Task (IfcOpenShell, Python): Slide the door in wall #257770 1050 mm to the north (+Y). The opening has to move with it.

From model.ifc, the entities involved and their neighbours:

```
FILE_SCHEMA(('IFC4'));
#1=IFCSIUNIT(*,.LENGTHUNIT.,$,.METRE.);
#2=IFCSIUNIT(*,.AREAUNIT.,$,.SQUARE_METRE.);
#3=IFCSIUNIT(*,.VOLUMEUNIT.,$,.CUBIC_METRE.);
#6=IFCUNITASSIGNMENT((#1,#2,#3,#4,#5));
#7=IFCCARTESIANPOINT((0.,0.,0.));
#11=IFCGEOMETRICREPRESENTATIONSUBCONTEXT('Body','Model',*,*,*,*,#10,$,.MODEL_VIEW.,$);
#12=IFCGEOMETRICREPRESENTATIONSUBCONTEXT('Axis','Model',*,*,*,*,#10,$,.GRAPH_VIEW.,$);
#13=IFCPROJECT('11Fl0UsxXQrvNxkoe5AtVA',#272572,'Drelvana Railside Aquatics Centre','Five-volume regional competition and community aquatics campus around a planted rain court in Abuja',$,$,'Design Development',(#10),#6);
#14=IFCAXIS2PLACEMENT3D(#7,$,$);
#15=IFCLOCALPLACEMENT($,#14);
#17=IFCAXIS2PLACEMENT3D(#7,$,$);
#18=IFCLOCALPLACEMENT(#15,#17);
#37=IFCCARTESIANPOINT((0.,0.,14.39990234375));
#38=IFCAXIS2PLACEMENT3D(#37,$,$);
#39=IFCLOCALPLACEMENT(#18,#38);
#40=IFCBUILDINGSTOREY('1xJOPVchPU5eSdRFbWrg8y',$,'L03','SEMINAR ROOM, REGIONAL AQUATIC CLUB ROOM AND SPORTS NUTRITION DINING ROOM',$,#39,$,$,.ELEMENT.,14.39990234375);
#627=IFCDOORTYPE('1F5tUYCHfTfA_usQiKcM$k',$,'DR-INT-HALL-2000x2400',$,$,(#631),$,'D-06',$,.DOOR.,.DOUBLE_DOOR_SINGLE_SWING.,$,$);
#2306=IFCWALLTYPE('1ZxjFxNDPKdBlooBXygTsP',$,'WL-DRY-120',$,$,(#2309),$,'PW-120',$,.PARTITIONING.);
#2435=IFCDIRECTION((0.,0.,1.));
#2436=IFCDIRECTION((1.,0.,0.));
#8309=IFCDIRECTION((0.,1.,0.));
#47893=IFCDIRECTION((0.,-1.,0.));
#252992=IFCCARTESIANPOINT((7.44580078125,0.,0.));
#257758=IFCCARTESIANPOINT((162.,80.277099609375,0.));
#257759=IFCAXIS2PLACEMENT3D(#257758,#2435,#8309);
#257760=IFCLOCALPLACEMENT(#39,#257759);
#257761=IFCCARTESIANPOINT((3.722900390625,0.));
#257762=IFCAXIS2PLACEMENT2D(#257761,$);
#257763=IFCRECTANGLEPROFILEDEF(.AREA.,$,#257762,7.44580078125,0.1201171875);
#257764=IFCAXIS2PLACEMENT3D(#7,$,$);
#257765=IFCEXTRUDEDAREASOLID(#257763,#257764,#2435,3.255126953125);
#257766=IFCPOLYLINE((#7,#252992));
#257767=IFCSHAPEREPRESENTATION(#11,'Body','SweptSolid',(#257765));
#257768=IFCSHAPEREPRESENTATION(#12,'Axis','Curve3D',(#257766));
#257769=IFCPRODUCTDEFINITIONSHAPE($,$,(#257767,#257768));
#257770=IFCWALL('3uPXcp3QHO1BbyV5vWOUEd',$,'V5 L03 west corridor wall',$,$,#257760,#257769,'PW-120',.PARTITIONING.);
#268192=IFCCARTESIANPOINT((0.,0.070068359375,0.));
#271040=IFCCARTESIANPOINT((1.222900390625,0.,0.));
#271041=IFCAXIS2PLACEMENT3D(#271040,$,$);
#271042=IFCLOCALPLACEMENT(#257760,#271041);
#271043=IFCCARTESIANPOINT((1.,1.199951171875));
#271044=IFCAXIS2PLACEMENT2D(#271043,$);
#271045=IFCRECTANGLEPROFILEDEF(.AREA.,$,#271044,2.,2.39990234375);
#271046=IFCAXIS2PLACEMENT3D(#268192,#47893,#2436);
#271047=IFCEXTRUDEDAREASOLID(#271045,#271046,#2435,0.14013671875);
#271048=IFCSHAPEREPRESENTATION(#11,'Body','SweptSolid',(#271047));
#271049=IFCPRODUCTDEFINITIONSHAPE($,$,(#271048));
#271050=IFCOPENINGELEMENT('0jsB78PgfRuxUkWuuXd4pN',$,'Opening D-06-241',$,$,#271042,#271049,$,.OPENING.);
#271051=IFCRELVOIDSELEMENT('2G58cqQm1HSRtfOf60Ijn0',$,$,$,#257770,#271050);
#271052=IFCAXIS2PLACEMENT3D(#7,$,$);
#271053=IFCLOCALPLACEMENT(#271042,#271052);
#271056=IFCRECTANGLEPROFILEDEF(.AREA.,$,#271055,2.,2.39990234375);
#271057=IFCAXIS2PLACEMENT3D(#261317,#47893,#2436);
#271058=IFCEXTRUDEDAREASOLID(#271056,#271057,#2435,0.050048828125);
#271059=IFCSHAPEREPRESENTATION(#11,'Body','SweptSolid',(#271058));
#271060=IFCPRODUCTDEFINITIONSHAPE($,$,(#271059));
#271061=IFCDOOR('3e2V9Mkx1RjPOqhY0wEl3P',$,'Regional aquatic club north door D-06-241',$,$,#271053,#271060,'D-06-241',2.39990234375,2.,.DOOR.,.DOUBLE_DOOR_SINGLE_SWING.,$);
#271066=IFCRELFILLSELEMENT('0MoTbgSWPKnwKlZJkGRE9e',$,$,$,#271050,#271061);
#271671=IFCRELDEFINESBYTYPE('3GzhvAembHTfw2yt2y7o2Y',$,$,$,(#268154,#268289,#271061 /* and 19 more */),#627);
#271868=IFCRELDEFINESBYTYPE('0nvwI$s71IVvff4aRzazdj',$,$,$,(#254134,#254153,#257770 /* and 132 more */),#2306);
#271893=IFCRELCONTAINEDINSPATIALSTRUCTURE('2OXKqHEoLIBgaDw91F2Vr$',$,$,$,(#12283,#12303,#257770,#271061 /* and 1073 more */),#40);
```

```python
import ifcopenshell
import ifcopenshell.api.geometry
import ifcopenshell.util.placement

model = ifcopenshell.open("model.ifc")

door = model.by_guid("3e2V9Mkx1RjPOqhY0wEl3P")
opening = door.FillsVoids[0].RelatingOpeningElement
wall = opening.VoidsElements[0].RelatingBuildingElement

wall_matrix = ifcopenshell.util.placement.get_local_placement(wall.ObjectPlacement)
shift = wall_matrix[:3, 0] * 1.05
before = ifcopenshell.util.placement.get_local_placement(door.ObjectPlacement)[:3, 3].copy()

# The door is placed relative to its opening, so it follows when the opening moves.
matrix = ifcopenshell.util.placement.get_local_placement(opening.ObjectPlacement)
matrix[:3, 3] += shift
ifcopenshell.api.geometry.edit_object_placement(
    model, product=opening, matrix=matrix, is_si=False, should_transform_children=True
)

after = ifcopenshell.util.placement.get_local_placement(door.ObjectPlacement)[:3, 3]
print("door moved by", (after - before).round(3) + 0.0)

model.write("model_edited.ifc")
```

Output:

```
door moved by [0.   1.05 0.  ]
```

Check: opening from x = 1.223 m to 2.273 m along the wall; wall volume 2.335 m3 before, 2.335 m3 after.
